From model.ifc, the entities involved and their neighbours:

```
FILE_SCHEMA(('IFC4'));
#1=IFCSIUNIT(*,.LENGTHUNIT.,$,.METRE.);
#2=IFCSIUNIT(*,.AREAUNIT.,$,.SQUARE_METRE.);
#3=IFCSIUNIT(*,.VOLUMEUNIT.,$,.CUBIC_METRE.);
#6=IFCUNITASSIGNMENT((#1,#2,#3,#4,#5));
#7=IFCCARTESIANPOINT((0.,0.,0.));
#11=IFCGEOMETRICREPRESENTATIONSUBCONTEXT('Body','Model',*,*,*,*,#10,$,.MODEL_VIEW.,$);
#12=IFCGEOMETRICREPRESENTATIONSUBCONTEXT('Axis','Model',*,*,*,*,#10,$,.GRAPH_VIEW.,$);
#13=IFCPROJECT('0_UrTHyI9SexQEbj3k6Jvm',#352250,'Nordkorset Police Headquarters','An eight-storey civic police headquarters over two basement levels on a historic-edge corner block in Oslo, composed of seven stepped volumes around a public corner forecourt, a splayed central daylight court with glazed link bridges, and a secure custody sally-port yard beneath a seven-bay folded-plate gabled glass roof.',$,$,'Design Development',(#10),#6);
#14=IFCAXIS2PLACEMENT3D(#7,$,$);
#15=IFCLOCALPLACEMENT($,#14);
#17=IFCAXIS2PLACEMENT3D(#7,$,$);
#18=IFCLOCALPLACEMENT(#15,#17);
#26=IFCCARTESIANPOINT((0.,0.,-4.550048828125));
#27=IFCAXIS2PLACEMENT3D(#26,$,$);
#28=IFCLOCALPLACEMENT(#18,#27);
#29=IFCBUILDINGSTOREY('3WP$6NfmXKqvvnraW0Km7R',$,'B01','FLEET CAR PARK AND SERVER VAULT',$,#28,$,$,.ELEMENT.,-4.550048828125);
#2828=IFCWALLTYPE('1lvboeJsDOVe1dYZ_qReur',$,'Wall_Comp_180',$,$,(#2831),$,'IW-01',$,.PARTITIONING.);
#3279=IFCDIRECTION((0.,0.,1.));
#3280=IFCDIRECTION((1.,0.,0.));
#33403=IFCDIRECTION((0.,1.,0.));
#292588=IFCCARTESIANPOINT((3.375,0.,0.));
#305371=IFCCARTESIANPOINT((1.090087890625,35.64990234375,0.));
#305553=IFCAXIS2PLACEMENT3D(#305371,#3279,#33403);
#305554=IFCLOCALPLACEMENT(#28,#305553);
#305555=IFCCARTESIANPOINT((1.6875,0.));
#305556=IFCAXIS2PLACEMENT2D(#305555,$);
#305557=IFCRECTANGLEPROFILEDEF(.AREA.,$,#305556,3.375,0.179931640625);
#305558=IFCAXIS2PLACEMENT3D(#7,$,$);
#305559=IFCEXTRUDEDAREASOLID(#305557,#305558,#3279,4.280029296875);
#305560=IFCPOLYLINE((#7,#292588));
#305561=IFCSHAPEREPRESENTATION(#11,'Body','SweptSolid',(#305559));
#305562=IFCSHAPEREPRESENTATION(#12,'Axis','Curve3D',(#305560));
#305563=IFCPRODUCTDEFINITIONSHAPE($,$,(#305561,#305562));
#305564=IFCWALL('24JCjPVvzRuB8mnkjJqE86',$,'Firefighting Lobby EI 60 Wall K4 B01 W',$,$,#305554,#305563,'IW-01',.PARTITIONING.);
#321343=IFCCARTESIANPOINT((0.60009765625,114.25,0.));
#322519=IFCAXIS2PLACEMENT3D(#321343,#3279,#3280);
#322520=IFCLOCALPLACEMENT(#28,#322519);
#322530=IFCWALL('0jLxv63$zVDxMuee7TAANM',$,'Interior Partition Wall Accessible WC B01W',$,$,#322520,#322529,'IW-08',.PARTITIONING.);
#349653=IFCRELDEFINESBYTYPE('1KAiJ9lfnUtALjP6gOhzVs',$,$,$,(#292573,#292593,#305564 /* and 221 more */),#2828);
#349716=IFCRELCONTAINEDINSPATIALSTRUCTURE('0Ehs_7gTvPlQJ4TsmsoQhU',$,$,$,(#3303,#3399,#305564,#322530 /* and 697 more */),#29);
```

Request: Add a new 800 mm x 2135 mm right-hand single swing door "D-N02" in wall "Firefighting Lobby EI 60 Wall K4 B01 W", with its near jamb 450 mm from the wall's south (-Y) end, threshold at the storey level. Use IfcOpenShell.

```python
import numpy as np
import ifcopenshell
import ifcopenshell.api.feature
import ifcopenshell.api.geometry
import ifcopenshell.api.root
import ifcopenshell.api.spatial
import ifcopenshell.geom
import ifcopenshell.util.element
import ifcopenshell.util.placement
import ifcopenshell.util.representation
import ifcopenshell.util.shape
import ifcopenshell.util.unit

model = ifcopenshell.open("model.ifc")
unit_scale = ifcopenshell.util.unit.calculate_unit_scale(model)
settings = ifcopenshell.geom.settings()


def volume(element):
    """Net volume in cubic metres, openings subtracted."""
    shape = ifcopenshell.geom.create_shape(settings, element)
    return ifcopenshell.util.shape.get_volume(shape.geometry)


wall = model.by_guid("24JCjPVvzRuB8mnkjJqE86")
storey = ifcopenshell.util.element.get_container(wall, ifc_class="IfcBuildingStorey")
context = ifcopenshell.util.representation.get_context(model, "Model", "Body", "MODEL_VIEW")
before = volume(wall)

width, height, from_end, sill = 0.8, 2.135, 0.45, 0.0  # metres

# The wall runs along its own X axis, and the end named is its -X end.
wall_shape = ifcopenshell.geom.create_shape(settings, wall)
x, y, z = ifcopenshell.util.shape.get_vertices(wall_shape.geometry).T
start = x.min() + from_end
face, thickness = float(y.min()), float(y.max() - y.min())
wall_matrix = ifcopenshell.util.placement.get_local_placement(wall.ObjectPlacement)
level = ifcopenshell.util.placement.get_local_placement(storey.ObjectPlacement)[2, 3]


def in_wall(x, y):
    """Placement at x, y metres in the wall's axes, at sill height."""
    matrix = wall_matrix.copy()
    matrix[:, 3] = wall_matrix @ np.array([x / unit_scale, y / unit_scale, 0.0, 1.0])
    matrix[2, 3] = level + sill / unit_scale
    return matrix


# Opening: a box that overshoots both wall faces by 50 mm.
opening = ifcopenshell.api.root.create_entity(model, ifc_class="IfcOpeningElement", predefined_type="OPENING")
box = ifcopenshell.api.geometry.add_wall_representation(
    model, context=context, length=width, height=height, thickness=thickness + 0.1
)
ifcopenshell.api.geometry.assign_representation(model, product=opening, representation=box)
ifcopenshell.api.geometry.edit_object_placement(model, product=opening, matrix=in_wall(start, face - 0.05), is_si=False)
ifcopenshell.api.feature.add_feature(model, feature=opening, element=wall)

door = ifcopenshell.api.root.create_entity(model, ifc_class="IfcDoor", name="D-N02", predefined_type="DOOR")
door.OverallWidth, door.OverallHeight = width / unit_scale, height / unit_scale
door.OperationType = "SINGLE_SWING_RIGHT"
body = ifcopenshell.api.geometry.add_door_representation(
    model,
    context=context,
    overall_width=door.OverallWidth,
    overall_height=door.OverallHeight,
    operation_type="SINGLE_SWING_RIGHT",
    lining_properties={"LiningDepth": thickness / unit_scale, "ThresholdDepth": thickness / unit_scale},
)
ifcopenshell.api.geometry.assign_representation(model, product=door, representation=body)
ifcopenshell.api.spatial.assign_container(model, products=[door], relating_structure=storey)
ifcopenshell.api.feature.add_filling(model, opening=opening, element=door)

# The lining spans the wall, so the door starts at the wall face.
ifcopenshell.api.geometry.edit_object_placement(model, product=door, matrix=in_wall(start, face), is_si=False)

after = volume(wall)

print(f"wall volume {before:.3f} -> {after:.3f} m3")

model.write("model_rev.ifc")
```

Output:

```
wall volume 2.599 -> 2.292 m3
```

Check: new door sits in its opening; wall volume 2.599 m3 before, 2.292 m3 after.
